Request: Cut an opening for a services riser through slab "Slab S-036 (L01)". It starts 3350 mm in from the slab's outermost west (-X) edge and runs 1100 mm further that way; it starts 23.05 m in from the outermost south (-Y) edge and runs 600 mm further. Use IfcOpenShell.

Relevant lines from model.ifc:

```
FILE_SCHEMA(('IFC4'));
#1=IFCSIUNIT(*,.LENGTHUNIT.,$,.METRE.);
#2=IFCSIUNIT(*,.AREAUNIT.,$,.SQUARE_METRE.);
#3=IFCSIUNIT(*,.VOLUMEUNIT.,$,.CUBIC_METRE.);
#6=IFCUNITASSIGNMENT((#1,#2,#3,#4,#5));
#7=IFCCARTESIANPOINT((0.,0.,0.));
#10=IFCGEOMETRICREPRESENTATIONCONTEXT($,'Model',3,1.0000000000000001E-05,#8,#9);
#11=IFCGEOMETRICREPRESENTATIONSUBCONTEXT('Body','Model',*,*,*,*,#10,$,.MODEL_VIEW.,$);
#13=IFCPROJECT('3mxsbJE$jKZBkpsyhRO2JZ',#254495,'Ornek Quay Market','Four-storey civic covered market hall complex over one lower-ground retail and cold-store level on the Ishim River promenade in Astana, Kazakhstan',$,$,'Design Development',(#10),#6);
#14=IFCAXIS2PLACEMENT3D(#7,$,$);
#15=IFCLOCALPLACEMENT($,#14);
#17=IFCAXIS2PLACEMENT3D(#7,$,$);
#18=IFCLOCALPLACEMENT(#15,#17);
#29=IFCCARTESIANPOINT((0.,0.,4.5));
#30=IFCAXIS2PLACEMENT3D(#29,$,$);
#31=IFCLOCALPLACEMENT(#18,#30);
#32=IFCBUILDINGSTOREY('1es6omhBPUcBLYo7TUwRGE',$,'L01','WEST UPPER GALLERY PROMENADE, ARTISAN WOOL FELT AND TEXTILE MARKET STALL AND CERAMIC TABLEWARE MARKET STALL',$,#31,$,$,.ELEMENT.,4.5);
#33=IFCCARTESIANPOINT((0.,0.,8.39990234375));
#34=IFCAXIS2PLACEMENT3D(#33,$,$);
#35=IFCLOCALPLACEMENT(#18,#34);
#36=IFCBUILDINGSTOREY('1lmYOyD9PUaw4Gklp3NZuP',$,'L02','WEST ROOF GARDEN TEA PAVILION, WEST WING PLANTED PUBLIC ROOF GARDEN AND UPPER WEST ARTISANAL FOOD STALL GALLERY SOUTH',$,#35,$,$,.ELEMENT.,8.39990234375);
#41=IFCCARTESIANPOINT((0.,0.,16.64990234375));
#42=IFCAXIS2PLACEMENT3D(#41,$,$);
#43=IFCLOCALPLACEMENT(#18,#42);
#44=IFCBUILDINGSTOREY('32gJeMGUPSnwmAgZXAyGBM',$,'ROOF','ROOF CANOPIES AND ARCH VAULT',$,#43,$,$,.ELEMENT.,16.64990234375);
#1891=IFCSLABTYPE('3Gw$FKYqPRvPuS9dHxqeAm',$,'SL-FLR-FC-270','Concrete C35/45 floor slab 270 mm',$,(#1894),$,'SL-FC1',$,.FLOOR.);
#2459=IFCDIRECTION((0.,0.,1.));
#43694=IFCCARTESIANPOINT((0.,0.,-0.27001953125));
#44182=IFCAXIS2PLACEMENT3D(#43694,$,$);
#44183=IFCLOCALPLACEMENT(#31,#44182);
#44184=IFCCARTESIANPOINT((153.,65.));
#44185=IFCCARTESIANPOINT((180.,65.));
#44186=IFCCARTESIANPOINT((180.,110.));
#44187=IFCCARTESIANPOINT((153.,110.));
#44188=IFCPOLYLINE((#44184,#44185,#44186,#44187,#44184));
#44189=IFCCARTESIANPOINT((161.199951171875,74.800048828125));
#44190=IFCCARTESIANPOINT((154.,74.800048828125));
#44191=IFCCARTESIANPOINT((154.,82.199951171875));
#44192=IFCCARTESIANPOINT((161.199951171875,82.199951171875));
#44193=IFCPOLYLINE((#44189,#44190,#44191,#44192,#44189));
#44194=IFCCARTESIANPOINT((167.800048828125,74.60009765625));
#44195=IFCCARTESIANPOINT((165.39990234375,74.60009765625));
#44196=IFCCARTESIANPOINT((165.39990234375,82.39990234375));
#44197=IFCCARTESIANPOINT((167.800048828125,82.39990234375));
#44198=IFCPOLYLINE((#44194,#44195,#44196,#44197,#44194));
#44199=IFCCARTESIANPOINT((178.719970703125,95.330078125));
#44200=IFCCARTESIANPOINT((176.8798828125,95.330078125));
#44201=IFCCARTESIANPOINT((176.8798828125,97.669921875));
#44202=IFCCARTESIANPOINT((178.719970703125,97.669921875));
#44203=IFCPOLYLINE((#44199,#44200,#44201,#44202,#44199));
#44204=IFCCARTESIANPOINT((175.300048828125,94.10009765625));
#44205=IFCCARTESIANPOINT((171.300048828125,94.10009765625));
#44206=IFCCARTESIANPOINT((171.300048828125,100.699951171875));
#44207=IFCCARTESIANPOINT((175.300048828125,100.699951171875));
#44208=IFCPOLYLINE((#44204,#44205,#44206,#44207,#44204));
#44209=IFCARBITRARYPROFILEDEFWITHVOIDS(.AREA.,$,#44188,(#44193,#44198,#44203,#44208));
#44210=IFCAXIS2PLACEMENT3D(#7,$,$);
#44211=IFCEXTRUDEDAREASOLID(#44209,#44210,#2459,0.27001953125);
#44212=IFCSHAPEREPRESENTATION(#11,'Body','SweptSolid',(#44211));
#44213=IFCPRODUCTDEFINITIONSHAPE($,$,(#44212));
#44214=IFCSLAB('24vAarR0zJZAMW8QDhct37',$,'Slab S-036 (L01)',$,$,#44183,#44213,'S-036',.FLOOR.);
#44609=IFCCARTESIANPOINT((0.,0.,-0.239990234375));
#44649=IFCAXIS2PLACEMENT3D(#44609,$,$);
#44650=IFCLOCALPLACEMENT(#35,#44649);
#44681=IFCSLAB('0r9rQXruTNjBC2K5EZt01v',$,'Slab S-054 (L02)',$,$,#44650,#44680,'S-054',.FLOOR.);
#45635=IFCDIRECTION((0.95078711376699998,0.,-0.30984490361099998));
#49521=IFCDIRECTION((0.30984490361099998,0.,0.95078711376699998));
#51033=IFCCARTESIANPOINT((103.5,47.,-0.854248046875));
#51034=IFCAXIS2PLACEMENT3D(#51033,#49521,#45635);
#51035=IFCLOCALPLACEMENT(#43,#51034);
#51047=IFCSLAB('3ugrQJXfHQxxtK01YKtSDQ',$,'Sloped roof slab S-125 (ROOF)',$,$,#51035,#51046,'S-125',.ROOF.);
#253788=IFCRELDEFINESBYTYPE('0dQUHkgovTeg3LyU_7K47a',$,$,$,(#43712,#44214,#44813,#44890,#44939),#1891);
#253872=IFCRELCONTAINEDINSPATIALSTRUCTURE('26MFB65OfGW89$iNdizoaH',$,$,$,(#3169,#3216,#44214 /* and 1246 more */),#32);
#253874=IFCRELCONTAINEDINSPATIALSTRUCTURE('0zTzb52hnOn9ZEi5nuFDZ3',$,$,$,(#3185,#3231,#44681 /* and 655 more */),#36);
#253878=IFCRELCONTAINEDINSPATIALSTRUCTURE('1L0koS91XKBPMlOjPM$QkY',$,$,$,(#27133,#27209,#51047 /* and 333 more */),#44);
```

```python
import numpy as np
import ifcopenshell
import ifcopenshell.api.feature
import ifcopenshell.api.geometry
import ifcopenshell.api.root
import ifcopenshell.geom
import ifcopenshell.util.placement
import ifcopenshell.util.representation
import ifcopenshell.util.shape
import ifcopenshell.util.unit

model = ifcopenshell.open("model.ifc")
unit_scale = ifcopenshell.util.unit.calculate_unit_scale(model)
settings = ifcopenshell.geom.settings()


def volume(element):
    """Net volume in cubic metres, openings subtracted."""
    shape = ifcopenshell.geom.create_shape(settings, element)
    return ifcopenshell.util.shape.get_volume(shape.geometry)


slab = model.by_guid("24vAarR0zJZAMW8QDhct37")
before = volume(slab)

# Extent in the slab's own axes, in metres. The edges named are its -X and -Y sides.
slab_shape = ifcopenshell.geom.create_shape(settings, slab)
vertices = ifcopenshell.util.shape.get_vertices(slab_shape.geometry)
x_min, y_min, bottom = vertices.min(axis=0)
top = vertices[:, 2].max()

opening = ifcopenshell.api.root.create_entity(model, ifc_class="IfcOpeningElement", name="Services riser opening", predefined_type="OPENING")
context = ifcopenshell.util.representation.get_context(model, "Model", "Body", "MODEL_VIEW")
width, depth = 1.1, 0.6
outline = [(0.0, 0.0), (width, 0.0), (width, depth), (0.0, depth), (0.0, 0.0)]
# Overshoot both faces by 50 mm so the cut is clean.
shape = ifcopenshell.api.geometry.add_slab_representation(
    model, context=context, depth=top - bottom + 0.1, polyline=outline
)
ifcopenshell.api.geometry.assign_representation(model, product=opening, representation=shape)

matrix = ifcopenshell.util.placement.get_local_placement(slab.ObjectPlacement)
matrix[:, 3] = matrix @ np.append(np.array([x_min + 3.35, y_min + 23.05, bottom - 0.05]) / unit_scale, 1.0)
ifcopenshell.api.geometry.edit_object_placement(model, product=opening, matrix=matrix, is_si=False)
ifcopenshell.api.feature.add_feature(model, feature=opening, element=slab)

after = volume(slab)

print(f"slab volume {before:.3f} -> {after:.3f} m3")

model.write("model_updated.ifc")
```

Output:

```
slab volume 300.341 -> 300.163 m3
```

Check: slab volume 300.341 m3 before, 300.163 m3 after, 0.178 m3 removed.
